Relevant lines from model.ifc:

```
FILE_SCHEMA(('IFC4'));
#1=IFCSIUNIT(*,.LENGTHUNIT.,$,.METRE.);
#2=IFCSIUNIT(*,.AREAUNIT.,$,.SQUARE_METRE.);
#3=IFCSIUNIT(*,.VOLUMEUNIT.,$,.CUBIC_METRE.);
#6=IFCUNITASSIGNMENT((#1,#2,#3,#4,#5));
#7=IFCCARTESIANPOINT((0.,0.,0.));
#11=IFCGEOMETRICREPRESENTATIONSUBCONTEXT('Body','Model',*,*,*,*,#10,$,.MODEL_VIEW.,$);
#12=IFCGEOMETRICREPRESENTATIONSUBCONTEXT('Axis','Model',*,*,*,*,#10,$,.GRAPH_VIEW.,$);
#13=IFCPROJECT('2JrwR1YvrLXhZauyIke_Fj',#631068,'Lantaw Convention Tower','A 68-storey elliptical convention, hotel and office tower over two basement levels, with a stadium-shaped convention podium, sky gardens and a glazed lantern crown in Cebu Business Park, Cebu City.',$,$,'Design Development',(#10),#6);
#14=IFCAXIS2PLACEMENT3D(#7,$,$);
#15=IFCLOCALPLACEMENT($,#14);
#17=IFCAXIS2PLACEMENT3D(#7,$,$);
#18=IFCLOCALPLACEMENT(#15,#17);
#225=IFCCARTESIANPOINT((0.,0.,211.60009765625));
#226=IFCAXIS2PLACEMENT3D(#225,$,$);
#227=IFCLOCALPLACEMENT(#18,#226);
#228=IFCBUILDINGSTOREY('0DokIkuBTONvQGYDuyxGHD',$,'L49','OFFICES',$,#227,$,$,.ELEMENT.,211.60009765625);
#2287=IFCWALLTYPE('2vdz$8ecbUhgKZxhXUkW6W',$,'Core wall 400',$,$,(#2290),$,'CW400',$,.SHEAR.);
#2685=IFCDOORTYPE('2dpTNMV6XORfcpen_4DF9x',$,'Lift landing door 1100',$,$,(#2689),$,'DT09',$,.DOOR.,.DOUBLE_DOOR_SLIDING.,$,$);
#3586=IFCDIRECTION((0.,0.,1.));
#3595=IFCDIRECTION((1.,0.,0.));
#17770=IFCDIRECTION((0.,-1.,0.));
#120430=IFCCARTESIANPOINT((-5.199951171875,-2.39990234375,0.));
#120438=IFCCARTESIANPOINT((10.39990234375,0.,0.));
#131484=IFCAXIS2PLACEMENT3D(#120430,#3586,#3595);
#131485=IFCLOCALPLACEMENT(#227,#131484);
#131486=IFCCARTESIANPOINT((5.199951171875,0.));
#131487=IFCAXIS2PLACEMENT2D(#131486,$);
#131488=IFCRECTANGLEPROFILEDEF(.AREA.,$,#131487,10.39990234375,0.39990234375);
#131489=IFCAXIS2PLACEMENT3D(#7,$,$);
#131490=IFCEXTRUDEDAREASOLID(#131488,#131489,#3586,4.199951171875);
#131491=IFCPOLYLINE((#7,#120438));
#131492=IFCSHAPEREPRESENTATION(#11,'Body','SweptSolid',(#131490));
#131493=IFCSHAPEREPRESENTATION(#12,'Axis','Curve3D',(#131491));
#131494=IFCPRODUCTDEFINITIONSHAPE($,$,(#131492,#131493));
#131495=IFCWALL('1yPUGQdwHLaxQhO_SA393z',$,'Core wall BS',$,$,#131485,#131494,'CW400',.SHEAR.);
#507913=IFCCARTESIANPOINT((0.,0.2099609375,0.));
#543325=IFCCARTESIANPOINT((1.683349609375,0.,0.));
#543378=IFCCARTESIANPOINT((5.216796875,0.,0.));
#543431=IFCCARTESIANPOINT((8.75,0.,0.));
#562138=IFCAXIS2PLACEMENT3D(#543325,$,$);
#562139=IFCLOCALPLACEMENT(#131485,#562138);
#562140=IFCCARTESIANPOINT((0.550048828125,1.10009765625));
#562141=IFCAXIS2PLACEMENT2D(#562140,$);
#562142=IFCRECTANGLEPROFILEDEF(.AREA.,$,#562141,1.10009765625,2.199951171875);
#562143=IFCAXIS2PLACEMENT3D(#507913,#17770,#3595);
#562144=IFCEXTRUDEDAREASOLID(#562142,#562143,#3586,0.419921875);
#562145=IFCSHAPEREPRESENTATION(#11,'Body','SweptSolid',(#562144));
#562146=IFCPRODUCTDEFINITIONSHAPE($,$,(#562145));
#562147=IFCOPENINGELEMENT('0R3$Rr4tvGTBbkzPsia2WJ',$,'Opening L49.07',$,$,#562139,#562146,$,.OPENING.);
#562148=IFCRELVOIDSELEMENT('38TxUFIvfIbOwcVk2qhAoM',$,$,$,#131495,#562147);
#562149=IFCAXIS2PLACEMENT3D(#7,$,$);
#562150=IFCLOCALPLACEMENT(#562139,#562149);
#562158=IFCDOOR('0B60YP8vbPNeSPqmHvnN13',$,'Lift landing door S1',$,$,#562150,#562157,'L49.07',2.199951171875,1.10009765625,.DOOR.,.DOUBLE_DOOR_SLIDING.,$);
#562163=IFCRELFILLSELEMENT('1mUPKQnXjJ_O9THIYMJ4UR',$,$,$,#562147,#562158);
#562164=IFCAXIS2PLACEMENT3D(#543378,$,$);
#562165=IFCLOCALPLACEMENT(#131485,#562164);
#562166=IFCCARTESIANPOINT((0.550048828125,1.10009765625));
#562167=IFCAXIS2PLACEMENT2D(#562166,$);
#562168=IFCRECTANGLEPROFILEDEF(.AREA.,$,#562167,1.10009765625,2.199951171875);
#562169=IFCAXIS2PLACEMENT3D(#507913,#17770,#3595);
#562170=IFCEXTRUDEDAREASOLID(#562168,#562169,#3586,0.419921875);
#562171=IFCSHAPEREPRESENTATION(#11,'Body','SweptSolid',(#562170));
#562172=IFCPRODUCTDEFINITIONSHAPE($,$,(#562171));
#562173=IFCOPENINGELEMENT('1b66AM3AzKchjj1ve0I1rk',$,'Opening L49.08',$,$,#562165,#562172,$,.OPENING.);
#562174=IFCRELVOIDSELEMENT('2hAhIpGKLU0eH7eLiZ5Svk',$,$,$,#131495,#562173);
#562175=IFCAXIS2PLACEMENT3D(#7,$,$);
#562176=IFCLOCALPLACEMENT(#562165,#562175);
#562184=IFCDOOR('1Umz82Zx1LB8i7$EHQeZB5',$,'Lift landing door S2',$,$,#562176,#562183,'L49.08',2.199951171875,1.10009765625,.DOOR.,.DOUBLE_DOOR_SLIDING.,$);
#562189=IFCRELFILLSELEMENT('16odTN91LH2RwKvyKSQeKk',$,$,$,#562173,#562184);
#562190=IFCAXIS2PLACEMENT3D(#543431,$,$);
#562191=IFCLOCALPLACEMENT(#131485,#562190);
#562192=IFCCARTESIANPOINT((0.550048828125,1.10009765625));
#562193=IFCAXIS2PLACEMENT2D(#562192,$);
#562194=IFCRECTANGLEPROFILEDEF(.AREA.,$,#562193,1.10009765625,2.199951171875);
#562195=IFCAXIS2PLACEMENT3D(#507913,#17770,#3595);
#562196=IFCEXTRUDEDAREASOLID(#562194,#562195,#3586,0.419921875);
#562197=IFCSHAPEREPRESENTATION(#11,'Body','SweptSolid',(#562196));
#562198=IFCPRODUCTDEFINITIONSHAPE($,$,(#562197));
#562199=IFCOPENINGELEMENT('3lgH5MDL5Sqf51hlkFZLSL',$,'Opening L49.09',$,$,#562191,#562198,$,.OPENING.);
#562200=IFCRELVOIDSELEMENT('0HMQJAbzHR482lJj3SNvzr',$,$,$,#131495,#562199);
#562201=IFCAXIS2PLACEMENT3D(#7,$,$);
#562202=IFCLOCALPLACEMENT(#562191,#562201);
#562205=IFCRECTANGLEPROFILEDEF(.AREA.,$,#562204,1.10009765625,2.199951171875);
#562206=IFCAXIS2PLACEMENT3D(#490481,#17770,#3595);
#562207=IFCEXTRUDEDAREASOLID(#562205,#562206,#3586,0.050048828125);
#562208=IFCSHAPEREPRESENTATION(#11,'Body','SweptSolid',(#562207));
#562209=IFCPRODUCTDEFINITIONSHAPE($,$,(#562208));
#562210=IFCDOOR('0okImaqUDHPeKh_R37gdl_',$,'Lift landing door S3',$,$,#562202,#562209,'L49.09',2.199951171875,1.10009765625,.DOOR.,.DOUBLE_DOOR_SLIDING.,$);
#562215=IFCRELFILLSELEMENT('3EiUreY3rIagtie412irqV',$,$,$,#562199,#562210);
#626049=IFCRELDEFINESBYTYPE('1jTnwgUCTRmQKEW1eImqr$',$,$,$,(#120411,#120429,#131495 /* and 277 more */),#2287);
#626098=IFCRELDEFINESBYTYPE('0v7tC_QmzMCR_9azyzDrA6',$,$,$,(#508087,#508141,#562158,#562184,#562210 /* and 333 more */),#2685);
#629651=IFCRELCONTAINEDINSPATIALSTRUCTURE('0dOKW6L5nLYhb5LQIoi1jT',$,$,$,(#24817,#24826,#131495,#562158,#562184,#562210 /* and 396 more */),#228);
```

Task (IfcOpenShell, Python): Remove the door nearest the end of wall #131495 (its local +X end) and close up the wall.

```python
import ifcopenshell
import ifcopenshell.api.feature
import ifcopenshell.api.root
import ifcopenshell.geom
import ifcopenshell.util.shape

model = ifcopenshell.open("model.ifc")
settings = ifcopenshell.geom.settings()


def volume(element):
    """Net volume in cubic metres, openings subtracted."""
    shape = ifcopenshell.geom.create_shape(settings, element)
    return ifcopenshell.util.shape.get_volume(shape.geometry)


door = model.by_guid("0okImaqUDHPeKh_R37gdl_")
opening = door.FillsVoids[0].RelatingOpeningElement
wall = opening.VoidsElements[0].RelatingBuildingElement
before = volume(wall)

ifcopenshell.api.root.remove_product(model, product=door)
ifcopenshell.api.feature.remove_feature(model, feature=opening)

after = volume(wall)

print(f"wall volume {before:.3f} -> {after:.3f} m3")

model.write("model_updated.ifc")
```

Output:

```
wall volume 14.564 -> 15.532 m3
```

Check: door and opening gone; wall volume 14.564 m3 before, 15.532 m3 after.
